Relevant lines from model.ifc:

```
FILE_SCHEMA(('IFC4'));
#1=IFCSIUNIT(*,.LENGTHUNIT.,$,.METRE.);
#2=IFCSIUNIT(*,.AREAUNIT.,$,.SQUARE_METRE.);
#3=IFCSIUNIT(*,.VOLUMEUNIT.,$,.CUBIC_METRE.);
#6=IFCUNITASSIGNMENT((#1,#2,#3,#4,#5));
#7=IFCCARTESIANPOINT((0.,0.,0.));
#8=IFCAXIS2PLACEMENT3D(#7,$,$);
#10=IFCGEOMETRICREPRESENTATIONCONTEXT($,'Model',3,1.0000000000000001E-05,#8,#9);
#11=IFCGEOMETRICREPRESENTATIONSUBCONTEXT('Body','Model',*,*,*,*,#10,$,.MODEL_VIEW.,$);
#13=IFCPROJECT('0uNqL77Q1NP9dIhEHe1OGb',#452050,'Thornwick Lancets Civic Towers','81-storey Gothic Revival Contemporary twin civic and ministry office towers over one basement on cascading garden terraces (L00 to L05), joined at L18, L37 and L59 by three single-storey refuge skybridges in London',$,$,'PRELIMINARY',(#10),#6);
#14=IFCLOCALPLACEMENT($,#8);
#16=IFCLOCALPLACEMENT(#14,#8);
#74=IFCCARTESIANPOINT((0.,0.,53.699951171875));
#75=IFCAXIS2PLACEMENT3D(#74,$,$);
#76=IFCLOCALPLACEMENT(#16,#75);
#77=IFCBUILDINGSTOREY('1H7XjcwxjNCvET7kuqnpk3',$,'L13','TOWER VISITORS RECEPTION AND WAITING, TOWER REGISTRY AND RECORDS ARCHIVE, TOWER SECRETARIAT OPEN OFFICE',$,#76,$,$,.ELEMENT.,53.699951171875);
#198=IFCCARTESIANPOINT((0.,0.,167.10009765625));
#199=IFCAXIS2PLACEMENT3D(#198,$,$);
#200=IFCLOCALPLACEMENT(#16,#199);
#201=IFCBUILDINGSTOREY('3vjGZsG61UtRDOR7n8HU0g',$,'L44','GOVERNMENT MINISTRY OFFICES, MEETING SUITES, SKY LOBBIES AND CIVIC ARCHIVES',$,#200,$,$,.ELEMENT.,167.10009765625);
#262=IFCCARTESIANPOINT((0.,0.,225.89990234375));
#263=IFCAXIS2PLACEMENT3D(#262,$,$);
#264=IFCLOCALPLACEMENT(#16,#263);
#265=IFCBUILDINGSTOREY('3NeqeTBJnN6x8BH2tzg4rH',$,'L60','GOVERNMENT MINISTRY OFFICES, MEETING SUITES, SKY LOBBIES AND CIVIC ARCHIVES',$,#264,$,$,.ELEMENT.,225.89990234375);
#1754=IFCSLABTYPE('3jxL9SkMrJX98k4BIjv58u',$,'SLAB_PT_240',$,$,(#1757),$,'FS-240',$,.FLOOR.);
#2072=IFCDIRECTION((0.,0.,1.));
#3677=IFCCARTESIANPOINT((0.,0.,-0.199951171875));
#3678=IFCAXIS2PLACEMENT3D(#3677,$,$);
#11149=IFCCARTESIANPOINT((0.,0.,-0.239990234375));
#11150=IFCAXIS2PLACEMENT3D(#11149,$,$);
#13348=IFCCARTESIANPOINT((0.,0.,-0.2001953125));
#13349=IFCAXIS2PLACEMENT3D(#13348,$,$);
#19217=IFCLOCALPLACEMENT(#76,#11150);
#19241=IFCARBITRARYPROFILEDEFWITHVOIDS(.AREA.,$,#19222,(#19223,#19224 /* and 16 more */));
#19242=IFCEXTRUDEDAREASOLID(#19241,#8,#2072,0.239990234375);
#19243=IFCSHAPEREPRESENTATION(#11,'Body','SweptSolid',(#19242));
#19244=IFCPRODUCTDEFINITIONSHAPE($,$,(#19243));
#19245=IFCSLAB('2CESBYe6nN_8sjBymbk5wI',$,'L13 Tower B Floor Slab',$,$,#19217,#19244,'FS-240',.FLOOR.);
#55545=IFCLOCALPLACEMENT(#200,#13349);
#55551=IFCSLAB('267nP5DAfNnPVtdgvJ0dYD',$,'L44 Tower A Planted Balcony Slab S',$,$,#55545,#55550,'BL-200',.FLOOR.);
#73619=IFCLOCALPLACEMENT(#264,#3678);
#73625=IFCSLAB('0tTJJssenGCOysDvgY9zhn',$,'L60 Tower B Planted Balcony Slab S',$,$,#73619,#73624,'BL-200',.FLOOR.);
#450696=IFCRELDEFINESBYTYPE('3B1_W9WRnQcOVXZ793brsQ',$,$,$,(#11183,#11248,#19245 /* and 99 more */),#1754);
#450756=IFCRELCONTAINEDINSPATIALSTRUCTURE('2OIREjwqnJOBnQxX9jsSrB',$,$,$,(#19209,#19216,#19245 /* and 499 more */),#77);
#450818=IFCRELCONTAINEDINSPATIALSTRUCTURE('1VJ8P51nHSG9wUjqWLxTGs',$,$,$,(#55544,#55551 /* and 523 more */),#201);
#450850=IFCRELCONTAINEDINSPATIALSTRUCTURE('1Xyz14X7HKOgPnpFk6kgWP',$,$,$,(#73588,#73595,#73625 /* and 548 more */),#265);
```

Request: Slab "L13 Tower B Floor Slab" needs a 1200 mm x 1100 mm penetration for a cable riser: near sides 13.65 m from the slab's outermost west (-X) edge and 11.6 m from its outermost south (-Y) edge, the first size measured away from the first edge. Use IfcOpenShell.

```python
import numpy as np
import ifcopenshell
import ifcopenshell.api.feature
import ifcopenshell.api.geometry
import ifcopenshell.api.root
import ifcopenshell.geom
import ifcopenshell.util.placement
import ifcopenshell.util.representation
import ifcopenshell.util.shape
import ifcopenshell.util.unit

model = ifcopenshell.open("model.ifc")
unit_scale = ifcopenshell.util.unit.calculate_unit_scale(model)
settings = ifcopenshell.geom.settings()


def volume(element):
    """Net volume in cubic metres, openings subtracted."""
    shape = ifcopenshell.geom.create_shape(settings, element)
    return ifcopenshell.util.shape.get_volume(shape.geometry)


slab = model.by_guid("2CESBYe6nN_8sjBymbk5wI")
before = volume(slab)

# Extent in the slab's own axes, in metres. The edges named are its -X and -Y sides.
slab_shape = ifcopenshell.geom.create_shape(settings, slab)
vertices = ifcopenshell.util.shape.get_vertices(slab_shape.geometry)
x_min, y_min, bottom = vertices.min(axis=0)
top = vertices[:, 2].max()

opening = ifcopenshell.api.root.create_entity(model, ifc_class="IfcOpeningElement", name="Cable riser opening", predefined_type="OPENING")
context = ifcopenshell.util.representation.get_context(model, "Model", "Body", "MODEL_VIEW")
width, depth = 1.2, 1.1
outline = [(0.0, 0.0), (width, 0.0), (width, depth), (0.0, depth), (0.0, 0.0)]
# Overshoot both faces by 50 mm so the cut is clean.
shape = ifcopenshell.api.geometry.add_slab_representation(
    model, context=context, depth=top - bottom + 0.1, polyline=outline
)
ifcopenshell.api.geometry.assign_representation(model, product=opening, representation=shape)

matrix = ifcopenshell.util.placement.get_local_placement(slab.ObjectPlacement)
matrix[:, 3] = matrix @ np.append(np.array([x_min + 13.65, y_min + 11.6, bottom - 0.05]) / unit_scale, 1.0)
ifcopenshell.api.geometry.edit_object_placement(model, product=opening, matrix=matrix, is_si=False)
ifcopenshell.api.feature.add_feature(model, feature=opening, element=slab)

after = volume(slab)

print(f"slab volume {before:.3f} -> {after:.3f} m3")

model.write("model_edited.ifc")
```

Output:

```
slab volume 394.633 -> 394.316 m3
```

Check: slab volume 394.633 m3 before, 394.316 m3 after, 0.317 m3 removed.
